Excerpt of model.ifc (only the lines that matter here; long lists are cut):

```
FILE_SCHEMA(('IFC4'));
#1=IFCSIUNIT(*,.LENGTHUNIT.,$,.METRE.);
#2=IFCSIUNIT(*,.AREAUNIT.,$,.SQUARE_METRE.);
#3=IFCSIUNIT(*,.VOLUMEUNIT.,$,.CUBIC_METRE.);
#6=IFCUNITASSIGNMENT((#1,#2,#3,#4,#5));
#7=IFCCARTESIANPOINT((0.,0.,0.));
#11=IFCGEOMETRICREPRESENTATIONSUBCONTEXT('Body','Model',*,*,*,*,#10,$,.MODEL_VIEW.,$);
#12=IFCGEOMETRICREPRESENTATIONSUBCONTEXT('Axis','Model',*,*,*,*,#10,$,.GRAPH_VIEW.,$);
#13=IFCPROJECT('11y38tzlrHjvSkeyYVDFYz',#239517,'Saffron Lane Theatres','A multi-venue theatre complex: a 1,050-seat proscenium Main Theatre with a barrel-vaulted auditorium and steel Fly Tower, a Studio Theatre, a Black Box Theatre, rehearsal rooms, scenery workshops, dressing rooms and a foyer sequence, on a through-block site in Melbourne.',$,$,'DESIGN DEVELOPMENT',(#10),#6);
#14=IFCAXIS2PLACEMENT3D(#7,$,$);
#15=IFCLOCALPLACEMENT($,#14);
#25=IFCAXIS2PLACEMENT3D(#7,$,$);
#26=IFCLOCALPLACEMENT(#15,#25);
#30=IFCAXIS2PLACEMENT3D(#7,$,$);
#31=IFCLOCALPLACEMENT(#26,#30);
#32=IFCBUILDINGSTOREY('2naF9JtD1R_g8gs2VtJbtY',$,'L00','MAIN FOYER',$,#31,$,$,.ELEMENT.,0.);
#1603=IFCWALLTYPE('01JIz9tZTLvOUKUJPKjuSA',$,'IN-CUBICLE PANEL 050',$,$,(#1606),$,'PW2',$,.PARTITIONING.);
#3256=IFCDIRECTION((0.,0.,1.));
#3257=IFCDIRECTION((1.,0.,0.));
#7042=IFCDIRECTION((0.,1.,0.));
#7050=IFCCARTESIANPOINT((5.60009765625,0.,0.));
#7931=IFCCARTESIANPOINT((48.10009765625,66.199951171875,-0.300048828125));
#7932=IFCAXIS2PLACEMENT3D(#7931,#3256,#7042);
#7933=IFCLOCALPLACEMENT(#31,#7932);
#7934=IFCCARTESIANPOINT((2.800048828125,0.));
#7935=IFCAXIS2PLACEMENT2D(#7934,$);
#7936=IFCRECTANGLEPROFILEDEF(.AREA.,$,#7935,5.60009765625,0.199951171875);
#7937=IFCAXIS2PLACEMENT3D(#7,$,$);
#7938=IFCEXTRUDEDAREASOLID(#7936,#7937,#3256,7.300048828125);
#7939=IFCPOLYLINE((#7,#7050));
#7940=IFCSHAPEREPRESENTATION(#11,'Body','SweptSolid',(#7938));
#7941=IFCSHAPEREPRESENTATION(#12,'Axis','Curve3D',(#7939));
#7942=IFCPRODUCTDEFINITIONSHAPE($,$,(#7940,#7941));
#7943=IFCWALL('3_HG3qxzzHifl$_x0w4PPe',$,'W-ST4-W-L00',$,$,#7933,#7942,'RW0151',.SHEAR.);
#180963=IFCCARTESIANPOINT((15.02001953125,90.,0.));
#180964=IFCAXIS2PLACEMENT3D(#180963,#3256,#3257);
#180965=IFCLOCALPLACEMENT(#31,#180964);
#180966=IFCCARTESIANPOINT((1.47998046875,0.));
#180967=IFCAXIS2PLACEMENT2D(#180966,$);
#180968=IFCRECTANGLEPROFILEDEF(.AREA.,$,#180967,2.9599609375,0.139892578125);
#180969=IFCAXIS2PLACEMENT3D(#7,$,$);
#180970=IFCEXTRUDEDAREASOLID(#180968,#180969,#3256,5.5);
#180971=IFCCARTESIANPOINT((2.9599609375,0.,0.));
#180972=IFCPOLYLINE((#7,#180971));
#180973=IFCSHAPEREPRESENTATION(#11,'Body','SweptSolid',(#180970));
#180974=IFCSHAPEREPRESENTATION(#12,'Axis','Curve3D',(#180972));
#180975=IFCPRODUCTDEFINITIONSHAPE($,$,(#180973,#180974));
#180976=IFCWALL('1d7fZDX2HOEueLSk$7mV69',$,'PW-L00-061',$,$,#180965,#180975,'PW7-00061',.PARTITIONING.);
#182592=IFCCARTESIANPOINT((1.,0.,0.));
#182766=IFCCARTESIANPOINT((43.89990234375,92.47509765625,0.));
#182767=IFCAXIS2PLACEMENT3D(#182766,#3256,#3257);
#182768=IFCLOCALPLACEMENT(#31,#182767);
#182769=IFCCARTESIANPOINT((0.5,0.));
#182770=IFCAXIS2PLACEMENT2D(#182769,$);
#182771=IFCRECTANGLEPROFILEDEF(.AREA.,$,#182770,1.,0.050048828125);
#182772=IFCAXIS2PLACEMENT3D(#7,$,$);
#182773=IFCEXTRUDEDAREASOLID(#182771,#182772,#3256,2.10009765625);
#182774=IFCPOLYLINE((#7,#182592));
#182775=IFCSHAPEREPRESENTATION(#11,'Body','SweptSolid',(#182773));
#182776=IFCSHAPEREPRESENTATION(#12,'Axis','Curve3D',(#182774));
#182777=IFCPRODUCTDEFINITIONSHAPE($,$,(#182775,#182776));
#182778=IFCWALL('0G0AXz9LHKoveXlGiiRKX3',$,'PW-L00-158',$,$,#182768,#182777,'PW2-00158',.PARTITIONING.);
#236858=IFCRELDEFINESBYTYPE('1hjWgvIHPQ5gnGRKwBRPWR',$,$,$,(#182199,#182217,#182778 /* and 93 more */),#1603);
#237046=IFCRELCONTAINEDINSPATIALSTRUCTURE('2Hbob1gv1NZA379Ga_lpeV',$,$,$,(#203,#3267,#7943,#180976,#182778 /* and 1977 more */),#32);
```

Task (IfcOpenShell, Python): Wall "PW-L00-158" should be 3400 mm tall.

```python
import ifcopenshell
import ifcopenshell.geom
import ifcopenshell.util.representation
import ifcopenshell.util.shape

model = ifcopenshell.open("model.ifc")
settings = ifcopenshell.geom.settings()


def volume(element):
    """Net volume in cubic metres, openings subtracted."""
    shape = ifcopenshell.geom.create_shape(settings, element)
    return ifcopenshell.util.shape.get_volume(shape.geometry)


wall = model.by_guid("0G0AXz9LHKoveXlGiiRKX3")
before = volume(wall)

body = ifcopenshell.util.representation.get_representation(wall, "Model", "Body")
solid = body.Items[0]
old_height = solid.Depth
solid.Depth = 3.4
after = volume(wall)

print(f"height {old_height:g} -> {solid.Depth:g}, volume {before:.3f} -> {after:.3f} m3")

model.write("model_edited.ifc")
```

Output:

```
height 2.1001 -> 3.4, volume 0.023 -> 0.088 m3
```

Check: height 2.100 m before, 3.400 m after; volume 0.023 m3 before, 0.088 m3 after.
